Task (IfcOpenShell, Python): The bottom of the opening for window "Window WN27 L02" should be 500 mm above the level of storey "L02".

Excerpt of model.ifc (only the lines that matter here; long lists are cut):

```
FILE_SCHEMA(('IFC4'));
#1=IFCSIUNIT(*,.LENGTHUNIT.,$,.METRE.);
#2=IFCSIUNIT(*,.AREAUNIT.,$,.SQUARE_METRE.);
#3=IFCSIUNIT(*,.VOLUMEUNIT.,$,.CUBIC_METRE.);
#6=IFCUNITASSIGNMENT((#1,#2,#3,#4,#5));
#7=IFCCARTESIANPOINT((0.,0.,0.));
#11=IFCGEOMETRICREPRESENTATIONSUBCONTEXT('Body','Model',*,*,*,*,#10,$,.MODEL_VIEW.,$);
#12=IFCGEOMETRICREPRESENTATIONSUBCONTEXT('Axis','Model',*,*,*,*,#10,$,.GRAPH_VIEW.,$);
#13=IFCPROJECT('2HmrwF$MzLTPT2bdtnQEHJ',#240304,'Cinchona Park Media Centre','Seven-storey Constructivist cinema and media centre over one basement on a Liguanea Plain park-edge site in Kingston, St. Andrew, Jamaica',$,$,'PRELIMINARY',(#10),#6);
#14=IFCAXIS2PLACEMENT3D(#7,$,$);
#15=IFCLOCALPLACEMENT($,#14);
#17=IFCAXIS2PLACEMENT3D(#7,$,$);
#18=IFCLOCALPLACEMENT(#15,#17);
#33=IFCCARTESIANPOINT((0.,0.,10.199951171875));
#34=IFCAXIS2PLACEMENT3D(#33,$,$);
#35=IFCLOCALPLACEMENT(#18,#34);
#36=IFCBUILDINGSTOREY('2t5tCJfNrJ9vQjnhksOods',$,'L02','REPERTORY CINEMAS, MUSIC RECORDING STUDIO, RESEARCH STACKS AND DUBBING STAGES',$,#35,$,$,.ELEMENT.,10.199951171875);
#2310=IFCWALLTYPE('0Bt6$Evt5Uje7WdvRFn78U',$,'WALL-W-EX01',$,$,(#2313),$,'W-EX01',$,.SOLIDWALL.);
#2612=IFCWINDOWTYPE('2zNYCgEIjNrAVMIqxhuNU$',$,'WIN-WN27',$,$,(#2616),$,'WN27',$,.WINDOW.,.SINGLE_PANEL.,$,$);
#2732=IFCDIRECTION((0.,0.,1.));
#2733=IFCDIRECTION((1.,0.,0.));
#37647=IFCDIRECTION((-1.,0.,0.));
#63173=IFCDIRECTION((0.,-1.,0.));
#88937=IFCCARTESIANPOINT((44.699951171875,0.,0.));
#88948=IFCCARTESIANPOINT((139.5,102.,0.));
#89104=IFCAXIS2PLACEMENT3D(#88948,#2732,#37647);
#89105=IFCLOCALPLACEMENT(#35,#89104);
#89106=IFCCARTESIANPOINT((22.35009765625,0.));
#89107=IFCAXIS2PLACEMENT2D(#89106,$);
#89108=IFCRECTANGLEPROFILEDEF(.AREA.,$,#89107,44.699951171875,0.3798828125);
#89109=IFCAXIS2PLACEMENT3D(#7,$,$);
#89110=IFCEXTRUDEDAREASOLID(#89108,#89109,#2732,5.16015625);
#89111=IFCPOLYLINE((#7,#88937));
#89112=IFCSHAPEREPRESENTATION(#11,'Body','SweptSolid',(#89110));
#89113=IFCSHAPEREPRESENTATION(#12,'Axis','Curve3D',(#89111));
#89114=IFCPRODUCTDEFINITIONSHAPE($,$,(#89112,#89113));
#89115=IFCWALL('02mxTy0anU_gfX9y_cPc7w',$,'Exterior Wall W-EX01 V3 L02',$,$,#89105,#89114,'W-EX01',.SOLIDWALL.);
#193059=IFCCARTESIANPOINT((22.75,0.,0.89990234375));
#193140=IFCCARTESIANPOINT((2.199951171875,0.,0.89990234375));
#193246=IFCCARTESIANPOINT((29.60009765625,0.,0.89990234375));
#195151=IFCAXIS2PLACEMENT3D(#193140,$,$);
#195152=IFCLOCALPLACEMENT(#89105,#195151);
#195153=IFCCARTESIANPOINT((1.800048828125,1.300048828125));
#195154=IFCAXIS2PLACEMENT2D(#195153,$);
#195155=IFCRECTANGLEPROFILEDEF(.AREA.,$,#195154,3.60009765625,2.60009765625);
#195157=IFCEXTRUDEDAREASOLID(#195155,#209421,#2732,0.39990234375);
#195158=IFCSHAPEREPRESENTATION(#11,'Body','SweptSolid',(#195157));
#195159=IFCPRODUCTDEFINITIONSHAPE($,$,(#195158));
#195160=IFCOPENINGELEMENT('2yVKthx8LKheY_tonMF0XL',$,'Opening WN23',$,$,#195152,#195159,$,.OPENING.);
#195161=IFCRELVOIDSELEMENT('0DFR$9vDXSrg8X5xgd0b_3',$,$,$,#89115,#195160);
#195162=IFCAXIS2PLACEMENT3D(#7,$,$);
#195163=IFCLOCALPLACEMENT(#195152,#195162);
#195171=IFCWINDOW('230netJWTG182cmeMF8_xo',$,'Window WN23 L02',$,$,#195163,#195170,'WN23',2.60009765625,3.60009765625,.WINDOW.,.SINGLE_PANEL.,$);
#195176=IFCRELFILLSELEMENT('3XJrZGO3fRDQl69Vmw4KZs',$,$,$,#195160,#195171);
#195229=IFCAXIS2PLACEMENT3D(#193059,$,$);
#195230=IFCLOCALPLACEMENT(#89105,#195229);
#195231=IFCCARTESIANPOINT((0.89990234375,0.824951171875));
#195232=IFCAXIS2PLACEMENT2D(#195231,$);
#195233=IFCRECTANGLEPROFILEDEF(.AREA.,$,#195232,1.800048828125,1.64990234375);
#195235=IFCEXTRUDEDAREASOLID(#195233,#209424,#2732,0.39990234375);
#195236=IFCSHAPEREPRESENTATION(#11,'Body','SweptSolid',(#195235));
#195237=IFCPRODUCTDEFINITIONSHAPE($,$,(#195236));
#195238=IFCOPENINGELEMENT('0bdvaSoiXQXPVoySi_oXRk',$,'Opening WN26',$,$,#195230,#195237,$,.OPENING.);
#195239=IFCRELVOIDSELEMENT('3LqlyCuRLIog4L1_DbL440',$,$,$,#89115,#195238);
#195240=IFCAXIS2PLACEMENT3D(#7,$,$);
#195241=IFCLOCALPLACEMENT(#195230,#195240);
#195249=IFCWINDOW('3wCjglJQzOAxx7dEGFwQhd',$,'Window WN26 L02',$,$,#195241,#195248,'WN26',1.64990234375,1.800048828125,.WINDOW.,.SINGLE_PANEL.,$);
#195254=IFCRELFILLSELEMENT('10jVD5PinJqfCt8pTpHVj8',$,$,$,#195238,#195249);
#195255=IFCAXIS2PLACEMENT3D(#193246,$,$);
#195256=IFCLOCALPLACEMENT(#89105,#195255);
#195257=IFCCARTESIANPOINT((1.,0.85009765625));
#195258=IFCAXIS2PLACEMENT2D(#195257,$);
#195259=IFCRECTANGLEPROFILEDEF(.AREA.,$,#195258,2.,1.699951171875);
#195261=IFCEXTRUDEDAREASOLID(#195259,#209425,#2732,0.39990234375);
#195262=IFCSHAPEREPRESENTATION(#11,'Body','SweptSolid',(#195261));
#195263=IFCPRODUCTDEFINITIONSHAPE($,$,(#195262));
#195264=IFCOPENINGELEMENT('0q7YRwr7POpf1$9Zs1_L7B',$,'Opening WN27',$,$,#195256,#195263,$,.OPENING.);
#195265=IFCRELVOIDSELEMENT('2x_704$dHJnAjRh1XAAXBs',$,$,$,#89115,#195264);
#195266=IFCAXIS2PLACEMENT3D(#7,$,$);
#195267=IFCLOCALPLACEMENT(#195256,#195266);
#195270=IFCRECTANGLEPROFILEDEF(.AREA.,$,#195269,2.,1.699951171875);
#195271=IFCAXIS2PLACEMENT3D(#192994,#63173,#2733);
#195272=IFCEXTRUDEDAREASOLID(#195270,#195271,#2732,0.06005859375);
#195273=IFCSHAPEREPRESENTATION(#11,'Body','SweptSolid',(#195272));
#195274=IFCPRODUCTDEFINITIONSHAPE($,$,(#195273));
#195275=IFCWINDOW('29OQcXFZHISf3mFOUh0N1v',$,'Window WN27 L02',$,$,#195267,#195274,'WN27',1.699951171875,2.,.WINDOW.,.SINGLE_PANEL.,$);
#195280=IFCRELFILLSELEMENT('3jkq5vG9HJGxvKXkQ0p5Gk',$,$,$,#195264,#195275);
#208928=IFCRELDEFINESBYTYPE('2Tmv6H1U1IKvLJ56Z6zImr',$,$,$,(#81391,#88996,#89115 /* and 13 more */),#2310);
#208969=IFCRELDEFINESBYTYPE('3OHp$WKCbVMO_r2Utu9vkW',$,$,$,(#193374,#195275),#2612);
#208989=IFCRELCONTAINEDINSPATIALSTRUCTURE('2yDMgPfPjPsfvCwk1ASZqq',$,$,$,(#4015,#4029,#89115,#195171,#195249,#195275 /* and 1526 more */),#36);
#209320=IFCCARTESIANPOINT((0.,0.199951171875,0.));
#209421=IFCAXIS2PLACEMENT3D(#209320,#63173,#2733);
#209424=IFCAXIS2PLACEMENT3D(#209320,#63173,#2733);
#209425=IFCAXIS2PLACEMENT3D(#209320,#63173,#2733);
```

```python
import numpy as np
import ifcopenshell
import ifcopenshell.api.geometry
import ifcopenshell.geom
import ifcopenshell.util.element
import ifcopenshell.util.placement
import ifcopenshell.util.shape
import ifcopenshell.util.unit

model = ifcopenshell.open("model.ifc")
unit_scale = ifcopenshell.util.unit.calculate_unit_scale(model)

window = model.by_guid("29OQcXFZHISf3mFOUh0N1v")
opening = window.FillsVoids[0].RelatingOpeningElement
storey = ifcopenshell.util.element.get_container(window, ifc_class="IfcBuildingStorey")
level = ifcopenshell.util.placement.get_local_placement(storey.ObjectPlacement)[2, 3]

# The opening's origin need not be at the sill, so measure its lowest point.
shape = ifcopenshell.geom.create_shape(ifcopenshell.geom.settings(), opening)
bottom = ifcopenshell.util.shape.get_shape_bottom_elevation(shape, shape.geometry) / unit_scale
dz = level + 0.5 - bottom

shift = np.array([0.0, 0.0, dz])
# The window is placed relative to its opening, so it follows when the opening moves.
matrix = ifcopenshell.util.placement.get_local_placement(opening.ObjectPlacement)
matrix[:3, 3] += shift
ifcopenshell.api.geometry.edit_object_placement(
    model, product=opening, matrix=matrix, is_si=False, should_transform_children=True
)

print(f"moved by {dz * unit_scale:+.3f} m")

model.write("model_updated.ifc")
```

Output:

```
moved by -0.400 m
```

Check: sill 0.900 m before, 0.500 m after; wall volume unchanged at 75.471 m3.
